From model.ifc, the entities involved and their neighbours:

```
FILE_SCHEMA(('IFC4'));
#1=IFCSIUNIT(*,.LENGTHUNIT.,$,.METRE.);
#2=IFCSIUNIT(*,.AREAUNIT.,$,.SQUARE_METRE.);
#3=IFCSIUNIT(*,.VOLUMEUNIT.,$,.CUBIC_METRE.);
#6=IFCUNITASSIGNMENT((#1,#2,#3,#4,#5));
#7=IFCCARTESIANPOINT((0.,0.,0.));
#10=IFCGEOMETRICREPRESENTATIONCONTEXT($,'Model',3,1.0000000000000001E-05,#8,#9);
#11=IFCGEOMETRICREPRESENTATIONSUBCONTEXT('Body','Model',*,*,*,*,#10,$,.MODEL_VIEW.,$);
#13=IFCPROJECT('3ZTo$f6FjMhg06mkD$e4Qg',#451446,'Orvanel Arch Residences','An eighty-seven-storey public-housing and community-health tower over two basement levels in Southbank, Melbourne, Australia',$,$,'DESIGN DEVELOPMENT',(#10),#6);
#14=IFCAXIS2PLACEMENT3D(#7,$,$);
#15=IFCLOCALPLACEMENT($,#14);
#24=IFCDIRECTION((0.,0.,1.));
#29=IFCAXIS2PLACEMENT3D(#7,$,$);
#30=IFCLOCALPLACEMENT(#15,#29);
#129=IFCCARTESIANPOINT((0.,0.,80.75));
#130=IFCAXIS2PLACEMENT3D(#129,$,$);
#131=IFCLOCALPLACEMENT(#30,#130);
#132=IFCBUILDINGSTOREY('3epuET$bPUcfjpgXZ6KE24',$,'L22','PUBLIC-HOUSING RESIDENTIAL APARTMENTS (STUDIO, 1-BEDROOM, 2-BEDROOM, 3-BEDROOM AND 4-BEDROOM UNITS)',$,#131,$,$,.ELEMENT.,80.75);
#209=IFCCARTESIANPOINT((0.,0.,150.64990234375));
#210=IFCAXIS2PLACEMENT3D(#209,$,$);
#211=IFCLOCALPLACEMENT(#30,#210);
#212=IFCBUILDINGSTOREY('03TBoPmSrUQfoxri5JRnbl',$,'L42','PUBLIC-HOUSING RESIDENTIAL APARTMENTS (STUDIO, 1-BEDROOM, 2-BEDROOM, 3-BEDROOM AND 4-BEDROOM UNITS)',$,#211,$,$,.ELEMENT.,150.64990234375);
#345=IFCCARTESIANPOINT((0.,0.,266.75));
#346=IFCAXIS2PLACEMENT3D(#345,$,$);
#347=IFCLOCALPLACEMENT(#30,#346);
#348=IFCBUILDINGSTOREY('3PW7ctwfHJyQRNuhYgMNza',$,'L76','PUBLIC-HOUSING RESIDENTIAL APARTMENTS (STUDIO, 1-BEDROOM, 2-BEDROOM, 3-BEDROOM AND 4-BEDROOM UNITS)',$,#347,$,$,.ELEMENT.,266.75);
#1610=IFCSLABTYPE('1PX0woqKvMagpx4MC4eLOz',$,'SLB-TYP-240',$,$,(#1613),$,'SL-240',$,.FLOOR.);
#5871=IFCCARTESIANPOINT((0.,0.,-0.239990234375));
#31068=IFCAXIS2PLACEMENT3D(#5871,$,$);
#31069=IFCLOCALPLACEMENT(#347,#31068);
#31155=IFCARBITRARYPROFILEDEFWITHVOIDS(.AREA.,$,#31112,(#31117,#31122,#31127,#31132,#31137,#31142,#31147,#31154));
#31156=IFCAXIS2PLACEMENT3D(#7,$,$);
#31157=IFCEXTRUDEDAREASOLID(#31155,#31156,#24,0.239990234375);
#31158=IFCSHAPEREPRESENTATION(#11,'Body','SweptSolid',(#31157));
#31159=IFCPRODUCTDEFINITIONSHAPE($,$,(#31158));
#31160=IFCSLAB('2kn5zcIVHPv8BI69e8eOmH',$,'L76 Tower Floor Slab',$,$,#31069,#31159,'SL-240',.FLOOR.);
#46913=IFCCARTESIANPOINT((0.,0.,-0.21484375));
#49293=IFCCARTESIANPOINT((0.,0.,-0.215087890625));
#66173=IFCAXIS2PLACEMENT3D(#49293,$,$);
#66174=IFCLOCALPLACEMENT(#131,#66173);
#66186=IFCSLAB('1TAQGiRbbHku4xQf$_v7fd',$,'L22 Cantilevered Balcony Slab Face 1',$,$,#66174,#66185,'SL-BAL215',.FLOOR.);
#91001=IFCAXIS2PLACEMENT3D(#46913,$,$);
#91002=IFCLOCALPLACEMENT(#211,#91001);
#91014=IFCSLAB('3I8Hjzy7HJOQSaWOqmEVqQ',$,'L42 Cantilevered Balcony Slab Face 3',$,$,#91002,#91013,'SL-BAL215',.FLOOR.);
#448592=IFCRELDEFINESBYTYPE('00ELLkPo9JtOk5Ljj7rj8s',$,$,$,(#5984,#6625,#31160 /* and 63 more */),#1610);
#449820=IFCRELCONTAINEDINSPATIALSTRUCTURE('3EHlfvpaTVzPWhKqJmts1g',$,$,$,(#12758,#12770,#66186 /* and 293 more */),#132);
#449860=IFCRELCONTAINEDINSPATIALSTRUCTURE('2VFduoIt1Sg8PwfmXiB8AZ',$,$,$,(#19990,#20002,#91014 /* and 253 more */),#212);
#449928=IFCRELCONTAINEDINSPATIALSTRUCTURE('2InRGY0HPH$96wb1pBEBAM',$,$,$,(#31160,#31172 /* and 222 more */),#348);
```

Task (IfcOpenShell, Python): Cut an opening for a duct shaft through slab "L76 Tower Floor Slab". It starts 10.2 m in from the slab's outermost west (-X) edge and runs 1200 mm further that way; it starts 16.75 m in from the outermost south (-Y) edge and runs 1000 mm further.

```python
import numpy as np
import ifcopenshell
import ifcopenshell.api.feature
import ifcopenshell.api.geometry
import ifcopenshell.api.root
import ifcopenshell.geom
import ifcopenshell.util.placement
import ifcopenshell.util.representation
import ifcopenshell.util.shape
import ifcopenshell.util.unit

model = ifcopenshell.open("model.ifc")
unit_scale = ifcopenshell.util.unit.calculate_unit_scale(model)
settings = ifcopenshell.geom.settings()


def volume(element):
    """Net volume in cubic metres, openings subtracted."""
    shape = ifcopenshell.geom.create_shape(settings, element)
    return ifcopenshell.util.shape.get_volume(shape.geometry)


slab = model.by_guid("2kn5zcIVHPv8BI69e8eOmH")
before = volume(slab)

# Extent in the slab's own axes, in metres. The edges named are its -X and -Y sides.
slab_shape = ifcopenshell.geom.create_shape(settings, slab)
vertices = ifcopenshell.util.shape.get_vertices(slab_shape.geometry)
x_min, y_min, bottom = vertices.min(axis=0)
top = vertices[:, 2].max()

opening = ifcopenshell.api.root.create_entity(model, ifc_class="IfcOpeningElement", name="Duct shaft opening", predefined_type="OPENING")
context = ifcopenshell.util.representation.get_context(model, "Model", "Body", "MODEL_VIEW")
width, depth = 1.2, 1
outline = [(0.0, 0.0), (width, 0.0), (width, depth), (0.0, depth), (0.0, 0.0)]
# Overshoot both faces by 50 mm so the cut is clean.
shape = ifcopenshell.api.geometry.add_slab_representation(
    model, context=context, depth=top - bottom + 0.1, polyline=outline
)
ifcopenshell.api.geometry.assign_representation(model, product=opening, representation=shape)

matrix = ifcopenshell.util.placement.get_local_placement(slab.ObjectPlacement)
matrix[:, 3] = matrix @ np.append(np.array([x_min + 10.2, y_min + 16.75, bottom - 0.05]) / unit_scale, 1.0)
ifcopenshell.api.geometry.edit_object_placement(model, product=opening, matrix=matrix, is_si=False)
ifcopenshell.api.feature.add_feature(model, feature=opening, element=slab)

after = volume(slab)

print(f"slab volume {before:.3f} -> {after:.3f} m3")

model.write("model_v2.ifc")
```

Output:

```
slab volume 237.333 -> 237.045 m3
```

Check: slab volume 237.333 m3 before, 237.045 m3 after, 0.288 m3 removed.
